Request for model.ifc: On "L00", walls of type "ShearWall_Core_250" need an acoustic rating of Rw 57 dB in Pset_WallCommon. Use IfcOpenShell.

First a look at what the model holds.

```python
import ifcopenshell
import ifcopenshell.util.element

model = ifcopenshell.open("model.ifc")
print(model.schema)
storey = next(s for s in model.by_type("IfcBuildingStorey") if s.Name == "L00")
walls = [e for e in ifcopenshell.util.element.get_decomposition(storey) if e.is_a("IfcWall")]
seen = {}
for e in walls:
    element_type = ifcopenshell.util.element.get_type(e)
    key = (element_type.Name if element_type != e and element_type else None, ifcopenshell.util.element.get_pset(e, "Pset_WallCommon", "AcousticRating"))
    seen[key] = seen.get(key, 0) + 1
for (name, value), count in sorted(seen.items(), key=str):
    print(count, "x", name, "|", value)
```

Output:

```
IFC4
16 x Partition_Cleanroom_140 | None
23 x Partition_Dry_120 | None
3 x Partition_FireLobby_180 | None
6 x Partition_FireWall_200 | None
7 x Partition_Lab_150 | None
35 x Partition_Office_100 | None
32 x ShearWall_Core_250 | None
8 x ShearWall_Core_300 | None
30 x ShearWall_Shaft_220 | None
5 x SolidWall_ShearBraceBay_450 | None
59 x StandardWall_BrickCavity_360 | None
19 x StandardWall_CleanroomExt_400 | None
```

```python
import ifcopenshell
import ifcopenshell.api.pset
import ifcopenshell.util.element

model = ifcopenshell.open("model.ifc")

storey = next(s for s in model.by_type("IfcBuildingStorey") if s.Name == "L00")
walls = [e for e in ifcopenshell.util.element.get_decomposition(storey) if e.is_a("IfcWall")]

count = 0
for e in walls:
    element_type = ifcopenshell.util.element.get_type(e)
    if element_type in (None, e) or element_type.Name != "ShearWall_Core_250":
        continue
    # add_pset returns the element's existing set when there is one.
    pset = ifcopenshell.api.pset.add_pset(model, product=e, name="Pset_WallCommon")
    ifcopenshell.api.pset.edit_pset(model, pset=pset, properties={"AcousticRating": "Rw 57 dB"})
    count += 1

print(count, "walls updated")

model.write("model-out.ifc")
```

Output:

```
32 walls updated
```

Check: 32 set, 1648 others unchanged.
